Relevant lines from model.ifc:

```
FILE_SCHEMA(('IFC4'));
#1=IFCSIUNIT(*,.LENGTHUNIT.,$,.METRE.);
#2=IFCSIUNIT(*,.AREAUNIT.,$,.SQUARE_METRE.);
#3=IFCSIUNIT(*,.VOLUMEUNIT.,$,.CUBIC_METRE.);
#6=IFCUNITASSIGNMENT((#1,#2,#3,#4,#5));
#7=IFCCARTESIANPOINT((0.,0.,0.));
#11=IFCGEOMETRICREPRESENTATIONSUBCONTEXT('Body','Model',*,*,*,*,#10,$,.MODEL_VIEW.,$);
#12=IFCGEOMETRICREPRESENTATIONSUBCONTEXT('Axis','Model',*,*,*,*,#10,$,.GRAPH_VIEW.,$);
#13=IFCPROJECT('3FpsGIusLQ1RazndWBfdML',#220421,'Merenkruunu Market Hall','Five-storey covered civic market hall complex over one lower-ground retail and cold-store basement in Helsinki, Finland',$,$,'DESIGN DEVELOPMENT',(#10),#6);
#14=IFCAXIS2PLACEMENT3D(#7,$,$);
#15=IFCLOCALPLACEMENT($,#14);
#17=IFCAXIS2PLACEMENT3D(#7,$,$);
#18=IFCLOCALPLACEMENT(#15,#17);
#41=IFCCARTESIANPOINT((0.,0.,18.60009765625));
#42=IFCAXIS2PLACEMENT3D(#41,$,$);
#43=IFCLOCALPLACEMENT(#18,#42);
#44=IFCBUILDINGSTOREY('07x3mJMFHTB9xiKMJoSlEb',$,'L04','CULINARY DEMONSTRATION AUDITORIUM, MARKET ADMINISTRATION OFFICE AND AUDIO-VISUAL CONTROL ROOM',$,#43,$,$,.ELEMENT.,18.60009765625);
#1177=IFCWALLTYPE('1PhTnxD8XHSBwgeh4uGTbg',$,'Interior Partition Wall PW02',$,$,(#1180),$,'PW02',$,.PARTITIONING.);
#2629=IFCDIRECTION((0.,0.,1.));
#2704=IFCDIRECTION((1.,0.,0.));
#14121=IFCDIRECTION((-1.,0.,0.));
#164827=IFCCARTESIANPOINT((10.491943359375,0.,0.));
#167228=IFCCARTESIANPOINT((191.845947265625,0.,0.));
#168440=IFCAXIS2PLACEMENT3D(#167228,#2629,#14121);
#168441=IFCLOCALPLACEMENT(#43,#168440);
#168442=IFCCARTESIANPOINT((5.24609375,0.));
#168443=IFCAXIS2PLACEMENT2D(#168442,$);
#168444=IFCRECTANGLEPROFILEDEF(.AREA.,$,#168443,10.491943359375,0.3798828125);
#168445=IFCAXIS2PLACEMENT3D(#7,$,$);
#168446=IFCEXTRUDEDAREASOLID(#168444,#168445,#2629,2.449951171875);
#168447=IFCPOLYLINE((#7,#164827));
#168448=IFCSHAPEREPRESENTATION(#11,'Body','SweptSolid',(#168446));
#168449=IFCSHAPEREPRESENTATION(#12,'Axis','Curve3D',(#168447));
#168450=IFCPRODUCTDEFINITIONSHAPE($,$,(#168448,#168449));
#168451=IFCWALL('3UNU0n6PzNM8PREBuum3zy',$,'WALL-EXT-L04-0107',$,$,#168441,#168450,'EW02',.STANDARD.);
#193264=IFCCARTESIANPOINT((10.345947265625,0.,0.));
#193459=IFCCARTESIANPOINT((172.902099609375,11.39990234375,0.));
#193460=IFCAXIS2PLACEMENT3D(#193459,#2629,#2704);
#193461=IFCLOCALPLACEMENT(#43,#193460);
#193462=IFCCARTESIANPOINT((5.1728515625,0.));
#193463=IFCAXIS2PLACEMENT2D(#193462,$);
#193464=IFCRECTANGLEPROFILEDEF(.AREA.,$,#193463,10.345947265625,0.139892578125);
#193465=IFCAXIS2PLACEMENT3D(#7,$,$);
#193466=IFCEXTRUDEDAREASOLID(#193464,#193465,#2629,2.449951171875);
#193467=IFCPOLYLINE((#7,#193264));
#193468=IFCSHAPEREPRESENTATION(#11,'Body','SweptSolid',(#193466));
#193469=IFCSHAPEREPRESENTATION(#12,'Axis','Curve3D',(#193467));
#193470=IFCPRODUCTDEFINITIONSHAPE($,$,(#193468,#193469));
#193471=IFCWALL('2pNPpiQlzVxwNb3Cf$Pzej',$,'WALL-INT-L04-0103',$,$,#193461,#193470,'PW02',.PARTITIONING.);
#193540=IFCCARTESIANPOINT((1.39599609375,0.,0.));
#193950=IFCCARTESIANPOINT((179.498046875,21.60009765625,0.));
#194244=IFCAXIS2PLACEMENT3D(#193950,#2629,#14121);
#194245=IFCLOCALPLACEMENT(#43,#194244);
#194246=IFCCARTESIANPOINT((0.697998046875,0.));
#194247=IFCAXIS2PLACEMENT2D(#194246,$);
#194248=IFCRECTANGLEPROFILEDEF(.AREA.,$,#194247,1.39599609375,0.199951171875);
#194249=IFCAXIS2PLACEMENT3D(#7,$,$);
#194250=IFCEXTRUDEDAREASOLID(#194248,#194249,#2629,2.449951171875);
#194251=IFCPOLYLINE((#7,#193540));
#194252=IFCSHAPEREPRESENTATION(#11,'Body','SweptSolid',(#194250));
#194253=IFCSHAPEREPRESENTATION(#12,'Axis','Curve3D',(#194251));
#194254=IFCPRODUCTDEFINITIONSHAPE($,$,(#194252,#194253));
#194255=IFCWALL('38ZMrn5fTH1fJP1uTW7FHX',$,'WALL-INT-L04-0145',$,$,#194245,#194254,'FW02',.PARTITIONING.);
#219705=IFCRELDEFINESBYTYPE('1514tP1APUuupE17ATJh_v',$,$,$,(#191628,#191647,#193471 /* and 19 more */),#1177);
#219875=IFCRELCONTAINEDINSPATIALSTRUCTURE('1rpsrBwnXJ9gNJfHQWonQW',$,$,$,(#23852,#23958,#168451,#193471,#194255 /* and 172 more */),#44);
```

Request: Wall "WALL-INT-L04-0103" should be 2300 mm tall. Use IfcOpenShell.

```python
import ifcopenshell
import ifcopenshell.geom
import ifcopenshell.util.representation
import ifcopenshell.util.shape
import ifcopenshell.util.unit

model = ifcopenshell.open("model.ifc")
unit_scale = ifcopenshell.util.unit.calculate_unit_scale(model)
settings = ifcopenshell.geom.settings()


def volume(element):
    """Net volume in cubic metres, openings subtracted."""
    shape = ifcopenshell.geom.create_shape(settings, element)
    return ifcopenshell.util.shape.get_volume(shape.geometry)


wall = model.by_guid("2pNPpiQlzVxwNb3Cf$Pzej")
before = volume(wall)

body = ifcopenshell.util.representation.get_representation(wall, "Model", "Body")
solid = body.Items[0]
old_height = solid.Depth
solid.Depth = 2.3 / unit_scale
after = volume(wall)

print(f"height {old_height:g} -> {solid.Depth:g}, volume {before:.3f} -> {after:.3f} m3")

model.write("model_v2.ifc")
```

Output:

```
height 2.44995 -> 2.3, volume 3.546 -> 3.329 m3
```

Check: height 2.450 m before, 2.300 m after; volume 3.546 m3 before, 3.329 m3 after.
